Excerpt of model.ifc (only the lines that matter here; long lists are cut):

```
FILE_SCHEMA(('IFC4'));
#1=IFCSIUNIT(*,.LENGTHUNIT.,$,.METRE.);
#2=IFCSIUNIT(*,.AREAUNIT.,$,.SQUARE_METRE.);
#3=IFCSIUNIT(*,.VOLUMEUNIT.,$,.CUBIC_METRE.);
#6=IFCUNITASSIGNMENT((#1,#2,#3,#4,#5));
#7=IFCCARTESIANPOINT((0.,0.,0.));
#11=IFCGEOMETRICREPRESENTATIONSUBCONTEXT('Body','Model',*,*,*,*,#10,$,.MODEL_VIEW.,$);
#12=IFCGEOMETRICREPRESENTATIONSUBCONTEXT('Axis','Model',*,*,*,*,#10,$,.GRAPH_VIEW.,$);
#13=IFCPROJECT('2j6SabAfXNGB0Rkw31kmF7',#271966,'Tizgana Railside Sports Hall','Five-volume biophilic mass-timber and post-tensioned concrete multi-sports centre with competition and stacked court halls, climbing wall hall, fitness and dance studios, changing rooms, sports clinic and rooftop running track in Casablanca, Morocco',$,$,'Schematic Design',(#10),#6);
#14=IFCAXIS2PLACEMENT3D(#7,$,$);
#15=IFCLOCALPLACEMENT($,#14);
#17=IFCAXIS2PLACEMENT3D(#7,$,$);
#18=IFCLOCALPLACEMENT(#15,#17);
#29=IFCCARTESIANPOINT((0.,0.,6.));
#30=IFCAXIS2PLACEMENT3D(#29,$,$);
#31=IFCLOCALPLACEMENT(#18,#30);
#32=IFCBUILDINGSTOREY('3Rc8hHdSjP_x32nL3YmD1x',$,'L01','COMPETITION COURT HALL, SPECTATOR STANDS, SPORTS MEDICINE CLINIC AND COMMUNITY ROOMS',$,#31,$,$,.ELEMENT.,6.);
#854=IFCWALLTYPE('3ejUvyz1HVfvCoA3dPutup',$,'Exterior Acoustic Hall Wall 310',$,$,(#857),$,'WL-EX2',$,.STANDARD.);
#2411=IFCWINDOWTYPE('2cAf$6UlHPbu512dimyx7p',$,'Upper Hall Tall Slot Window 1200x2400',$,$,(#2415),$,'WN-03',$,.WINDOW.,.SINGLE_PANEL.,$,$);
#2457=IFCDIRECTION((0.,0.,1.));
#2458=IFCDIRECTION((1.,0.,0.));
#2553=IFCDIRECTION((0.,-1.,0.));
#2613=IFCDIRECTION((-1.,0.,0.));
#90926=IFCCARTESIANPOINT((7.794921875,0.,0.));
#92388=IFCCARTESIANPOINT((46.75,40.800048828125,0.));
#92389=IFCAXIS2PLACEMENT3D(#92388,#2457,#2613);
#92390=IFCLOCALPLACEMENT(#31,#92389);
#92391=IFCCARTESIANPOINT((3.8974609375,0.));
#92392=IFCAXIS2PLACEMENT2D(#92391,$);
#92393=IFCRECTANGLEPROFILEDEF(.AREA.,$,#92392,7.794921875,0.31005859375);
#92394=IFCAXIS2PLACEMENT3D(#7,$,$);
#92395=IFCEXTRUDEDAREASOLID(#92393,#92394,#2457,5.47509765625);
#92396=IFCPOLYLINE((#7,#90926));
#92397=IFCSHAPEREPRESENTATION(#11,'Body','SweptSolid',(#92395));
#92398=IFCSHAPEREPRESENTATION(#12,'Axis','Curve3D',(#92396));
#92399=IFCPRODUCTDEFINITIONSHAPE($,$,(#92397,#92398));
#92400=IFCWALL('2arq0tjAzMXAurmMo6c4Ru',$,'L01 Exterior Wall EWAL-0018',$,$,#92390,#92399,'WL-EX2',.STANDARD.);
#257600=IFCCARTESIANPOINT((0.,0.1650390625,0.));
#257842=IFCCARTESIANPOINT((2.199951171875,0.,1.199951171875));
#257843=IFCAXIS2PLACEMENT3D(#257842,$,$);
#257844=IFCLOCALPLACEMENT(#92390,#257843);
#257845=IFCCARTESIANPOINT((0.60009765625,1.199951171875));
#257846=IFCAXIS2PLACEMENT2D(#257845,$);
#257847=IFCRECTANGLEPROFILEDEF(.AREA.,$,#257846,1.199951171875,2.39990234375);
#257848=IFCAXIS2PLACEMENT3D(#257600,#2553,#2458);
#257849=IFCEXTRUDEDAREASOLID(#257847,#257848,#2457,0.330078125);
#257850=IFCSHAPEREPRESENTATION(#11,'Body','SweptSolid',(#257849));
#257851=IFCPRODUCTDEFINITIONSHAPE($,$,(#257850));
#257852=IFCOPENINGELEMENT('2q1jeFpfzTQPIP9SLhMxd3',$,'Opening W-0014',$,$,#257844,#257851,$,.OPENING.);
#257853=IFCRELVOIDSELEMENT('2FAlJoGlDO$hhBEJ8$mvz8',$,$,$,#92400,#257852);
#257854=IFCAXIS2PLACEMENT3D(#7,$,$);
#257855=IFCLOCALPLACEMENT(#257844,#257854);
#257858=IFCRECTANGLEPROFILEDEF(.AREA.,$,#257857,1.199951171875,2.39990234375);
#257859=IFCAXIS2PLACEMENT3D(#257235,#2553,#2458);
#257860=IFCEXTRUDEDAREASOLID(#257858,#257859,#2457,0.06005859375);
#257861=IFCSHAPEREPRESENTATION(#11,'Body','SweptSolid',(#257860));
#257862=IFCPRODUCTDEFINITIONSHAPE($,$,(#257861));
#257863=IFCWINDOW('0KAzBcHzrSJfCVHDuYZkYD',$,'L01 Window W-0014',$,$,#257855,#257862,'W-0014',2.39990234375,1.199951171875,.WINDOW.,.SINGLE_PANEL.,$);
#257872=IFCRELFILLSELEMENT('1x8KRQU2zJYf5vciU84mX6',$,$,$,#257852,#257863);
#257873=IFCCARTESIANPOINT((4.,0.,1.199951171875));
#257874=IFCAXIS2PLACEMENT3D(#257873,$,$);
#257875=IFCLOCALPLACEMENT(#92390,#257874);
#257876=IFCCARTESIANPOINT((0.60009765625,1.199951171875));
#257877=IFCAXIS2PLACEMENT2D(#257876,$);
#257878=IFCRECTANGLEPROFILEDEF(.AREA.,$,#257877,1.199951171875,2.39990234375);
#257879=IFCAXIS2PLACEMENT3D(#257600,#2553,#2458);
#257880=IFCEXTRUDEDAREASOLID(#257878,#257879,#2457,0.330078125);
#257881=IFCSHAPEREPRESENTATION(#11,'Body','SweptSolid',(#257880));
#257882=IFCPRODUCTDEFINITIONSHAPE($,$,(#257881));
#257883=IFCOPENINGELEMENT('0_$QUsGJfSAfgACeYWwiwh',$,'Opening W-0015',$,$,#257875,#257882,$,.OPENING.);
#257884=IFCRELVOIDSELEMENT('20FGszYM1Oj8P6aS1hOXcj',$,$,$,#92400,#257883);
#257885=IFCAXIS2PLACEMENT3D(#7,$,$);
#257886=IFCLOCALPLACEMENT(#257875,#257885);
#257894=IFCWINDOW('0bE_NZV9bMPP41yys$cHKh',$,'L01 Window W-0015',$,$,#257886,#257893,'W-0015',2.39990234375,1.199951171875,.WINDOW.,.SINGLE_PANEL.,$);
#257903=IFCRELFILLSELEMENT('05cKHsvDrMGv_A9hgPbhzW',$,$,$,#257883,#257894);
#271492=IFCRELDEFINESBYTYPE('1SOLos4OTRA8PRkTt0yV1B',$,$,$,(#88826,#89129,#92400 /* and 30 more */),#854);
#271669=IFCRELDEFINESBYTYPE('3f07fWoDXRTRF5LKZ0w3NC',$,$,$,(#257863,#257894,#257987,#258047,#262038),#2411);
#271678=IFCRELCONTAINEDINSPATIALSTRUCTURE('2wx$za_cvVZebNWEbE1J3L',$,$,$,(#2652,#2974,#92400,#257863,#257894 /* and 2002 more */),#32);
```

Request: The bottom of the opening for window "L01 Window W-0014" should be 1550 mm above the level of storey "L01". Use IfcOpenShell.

```python
import numpy as np
import ifcopenshell
import ifcopenshell.api.geometry
import ifcopenshell.geom
import ifcopenshell.util.element
import ifcopenshell.util.placement
import ifcopenshell.util.shape
import ifcopenshell.util.unit

model = ifcopenshell.open("model.ifc")
unit_scale = ifcopenshell.util.unit.calculate_unit_scale(model)

window = model.by_guid("0KAzBcHzrSJfCVHDuYZkYD")
opening = window.FillsVoids[0].RelatingOpeningElement
storey = ifcopenshell.util.element.get_container(window, ifc_class="IfcBuildingStorey")
level = ifcopenshell.util.placement.get_local_placement(storey.ObjectPlacement)[2, 3]

# The opening's origin need not be at the sill, so measure its lowest point.
shape = ifcopenshell.geom.create_shape(ifcopenshell.geom.settings(), opening)
bottom = ifcopenshell.util.shape.get_shape_bottom_elevation(shape, shape.geometry) / unit_scale
dz = level + 1.55 - bottom

shift = np.array([0.0, 0.0, dz])
# The window is placed relative to its opening, so it follows when the opening moves.
matrix = ifcopenshell.util.placement.get_local_placement(opening.ObjectPlacement)
matrix[:3, 3] += shift
ifcopenshell.api.geometry.edit_object_placement(
    model, product=opening, matrix=matrix, is_si=False, should_transform_children=True
)

print(f"moved by {dz * unit_scale:+.3f} m")

model.write("model_edited.ifc")
```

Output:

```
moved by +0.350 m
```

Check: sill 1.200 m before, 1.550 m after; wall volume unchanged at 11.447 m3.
